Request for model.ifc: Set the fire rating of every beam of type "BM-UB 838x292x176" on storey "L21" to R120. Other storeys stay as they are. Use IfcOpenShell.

First a look at what the model holds.

```python
import ifcopenshell
import ifcopenshell.util.element

model = ifcopenshell.open("model.ifc")
print(model.schema)
storey = next(s for s in model.by_type("IfcBuildingStorey") if s.Name == "L21")
beams = [e for e in ifcopenshell.util.element.get_decomposition(storey) if e.is_a("IfcBeam")]
seen = {}
for e in beams:
    element_type = ifcopenshell.util.element.get_type(e)
    key = (element_type.Name if element_type != e and element_type else None, ifcopenshell.util.element.get_pset(e, "Pset_BeamCommon", "FireRating"))
    seen[key] = seen.get(key, 0) + 1
for (name, value), count in sorted(seen.items(), key=str):
    print(count, "x", name, "|", value)
```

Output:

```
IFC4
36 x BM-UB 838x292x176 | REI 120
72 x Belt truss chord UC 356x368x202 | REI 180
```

```python
import ifcopenshell
import ifcopenshell.api.pset
import ifcopenshell.util.element

model = ifcopenshell.open("model.ifc")

storey = next(s for s in model.by_type("IfcBuildingStorey") if s.Name == "L21")
beams = [e for e in ifcopenshell.util.element.get_decomposition(storey) if e.is_a("IfcBeam")]

count = 0
for e in beams:
    element_type = ifcopenshell.util.element.get_type(e)
    if element_type in (None, e) or element_type.Name != "BM-UB 838x292x176":
        continue
    # add_pset returns the element's existing set when there is one.
    pset = ifcopenshell.api.pset.add_pset(model, product=e, name="Pset_BeamCommon")
    ifcopenshell.api.pset.edit_pset(model, pset=pset, properties={"FireRating": "R120"})
    count += 1

print(count, "beams updated")

model.write("model_rev.ifc")
```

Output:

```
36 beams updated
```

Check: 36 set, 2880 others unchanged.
